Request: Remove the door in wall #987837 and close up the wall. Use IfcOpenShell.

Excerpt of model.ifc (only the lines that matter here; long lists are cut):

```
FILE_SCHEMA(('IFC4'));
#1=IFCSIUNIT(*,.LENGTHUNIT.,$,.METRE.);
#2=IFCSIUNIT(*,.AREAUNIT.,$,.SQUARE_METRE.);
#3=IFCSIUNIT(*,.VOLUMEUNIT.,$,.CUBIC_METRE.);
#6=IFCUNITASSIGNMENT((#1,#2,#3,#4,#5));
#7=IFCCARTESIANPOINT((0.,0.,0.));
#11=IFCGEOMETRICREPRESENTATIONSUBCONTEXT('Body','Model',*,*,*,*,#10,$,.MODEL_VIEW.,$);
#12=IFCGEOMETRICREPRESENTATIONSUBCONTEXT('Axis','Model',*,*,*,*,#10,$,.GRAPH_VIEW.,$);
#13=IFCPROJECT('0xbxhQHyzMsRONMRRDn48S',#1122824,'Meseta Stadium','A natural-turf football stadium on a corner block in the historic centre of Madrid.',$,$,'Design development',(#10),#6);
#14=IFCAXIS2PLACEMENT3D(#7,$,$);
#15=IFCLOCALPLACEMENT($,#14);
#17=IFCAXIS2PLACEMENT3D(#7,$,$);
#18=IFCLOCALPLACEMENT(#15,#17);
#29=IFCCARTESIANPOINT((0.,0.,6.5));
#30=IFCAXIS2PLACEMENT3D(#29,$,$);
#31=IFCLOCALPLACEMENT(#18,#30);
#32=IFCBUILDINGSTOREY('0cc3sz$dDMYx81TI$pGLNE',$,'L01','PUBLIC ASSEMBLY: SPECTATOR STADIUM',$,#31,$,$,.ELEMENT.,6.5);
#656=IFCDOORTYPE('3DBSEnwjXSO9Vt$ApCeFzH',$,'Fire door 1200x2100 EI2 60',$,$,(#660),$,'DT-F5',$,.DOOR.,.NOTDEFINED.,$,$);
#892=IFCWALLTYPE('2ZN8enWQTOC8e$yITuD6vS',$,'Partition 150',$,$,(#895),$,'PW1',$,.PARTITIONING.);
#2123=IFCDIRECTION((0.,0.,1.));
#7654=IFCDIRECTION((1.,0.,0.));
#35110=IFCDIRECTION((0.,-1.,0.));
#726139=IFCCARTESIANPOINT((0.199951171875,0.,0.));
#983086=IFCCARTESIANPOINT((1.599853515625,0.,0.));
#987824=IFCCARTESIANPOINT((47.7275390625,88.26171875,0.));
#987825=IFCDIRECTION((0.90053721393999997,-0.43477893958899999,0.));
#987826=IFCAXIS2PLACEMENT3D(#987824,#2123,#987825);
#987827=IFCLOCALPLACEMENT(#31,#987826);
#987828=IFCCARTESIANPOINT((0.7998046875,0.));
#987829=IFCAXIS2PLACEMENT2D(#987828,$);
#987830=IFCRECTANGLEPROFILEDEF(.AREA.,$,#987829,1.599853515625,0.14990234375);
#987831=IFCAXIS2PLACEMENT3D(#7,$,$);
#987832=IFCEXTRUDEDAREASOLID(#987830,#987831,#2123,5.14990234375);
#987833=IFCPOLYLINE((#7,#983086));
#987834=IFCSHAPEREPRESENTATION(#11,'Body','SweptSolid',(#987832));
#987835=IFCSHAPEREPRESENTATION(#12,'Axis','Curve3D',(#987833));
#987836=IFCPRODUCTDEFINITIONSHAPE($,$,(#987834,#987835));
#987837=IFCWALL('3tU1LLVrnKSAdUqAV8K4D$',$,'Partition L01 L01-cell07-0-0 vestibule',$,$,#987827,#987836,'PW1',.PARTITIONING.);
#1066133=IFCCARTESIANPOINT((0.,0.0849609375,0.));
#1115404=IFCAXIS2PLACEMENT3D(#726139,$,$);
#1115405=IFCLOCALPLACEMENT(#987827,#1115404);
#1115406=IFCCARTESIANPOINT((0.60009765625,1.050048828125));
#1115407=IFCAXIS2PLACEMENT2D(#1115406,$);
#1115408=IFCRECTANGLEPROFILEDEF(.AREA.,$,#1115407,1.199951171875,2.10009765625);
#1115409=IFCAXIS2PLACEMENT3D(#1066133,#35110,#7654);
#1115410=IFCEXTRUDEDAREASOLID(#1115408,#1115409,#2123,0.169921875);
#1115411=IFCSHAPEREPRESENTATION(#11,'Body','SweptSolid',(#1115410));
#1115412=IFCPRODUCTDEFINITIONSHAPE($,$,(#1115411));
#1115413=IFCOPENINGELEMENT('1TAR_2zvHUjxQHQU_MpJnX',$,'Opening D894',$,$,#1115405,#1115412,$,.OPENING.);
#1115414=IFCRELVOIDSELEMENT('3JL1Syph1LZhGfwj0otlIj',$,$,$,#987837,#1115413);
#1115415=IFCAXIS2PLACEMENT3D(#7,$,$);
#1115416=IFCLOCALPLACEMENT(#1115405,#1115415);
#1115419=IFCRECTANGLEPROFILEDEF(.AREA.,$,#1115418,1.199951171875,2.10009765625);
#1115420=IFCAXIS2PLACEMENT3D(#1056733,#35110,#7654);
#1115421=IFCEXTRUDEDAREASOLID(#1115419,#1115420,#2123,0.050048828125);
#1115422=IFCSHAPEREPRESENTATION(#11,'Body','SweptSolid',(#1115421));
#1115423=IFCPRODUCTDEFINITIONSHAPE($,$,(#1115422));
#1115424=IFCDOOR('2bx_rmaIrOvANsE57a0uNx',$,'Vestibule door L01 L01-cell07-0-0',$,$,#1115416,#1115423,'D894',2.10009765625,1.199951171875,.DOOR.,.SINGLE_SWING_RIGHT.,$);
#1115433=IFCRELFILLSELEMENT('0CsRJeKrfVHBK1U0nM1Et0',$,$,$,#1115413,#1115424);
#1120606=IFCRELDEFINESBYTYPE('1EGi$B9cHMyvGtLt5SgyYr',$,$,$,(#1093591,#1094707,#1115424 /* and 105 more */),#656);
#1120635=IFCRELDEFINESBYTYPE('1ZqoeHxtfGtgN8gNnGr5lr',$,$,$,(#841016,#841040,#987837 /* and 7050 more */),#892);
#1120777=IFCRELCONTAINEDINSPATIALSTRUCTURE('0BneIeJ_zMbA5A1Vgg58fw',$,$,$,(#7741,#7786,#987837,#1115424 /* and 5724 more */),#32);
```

```python
import ifcopenshell
import ifcopenshell.api.feature
import ifcopenshell.api.root
import ifcopenshell.geom
import ifcopenshell.util.shape

model = ifcopenshell.open("model.ifc")
settings = ifcopenshell.geom.settings()


def volume(element):
    """Net volume in cubic metres, openings subtracted."""
    shape = ifcopenshell.geom.create_shape(settings, element)
    return ifcopenshell.util.shape.get_volume(shape.geometry)


door = model.by_guid("2bx_rmaIrOvANsE57a0uNx")
opening = door.FillsVoids[0].RelatingOpeningElement
wall = opening.VoidsElements[0].RelatingBuildingElement
before = volume(wall)

ifcopenshell.api.root.remove_product(model, product=door)
ifcopenshell.api.feature.remove_feature(model, feature=opening)

after = volume(wall)

print(f"wall volume {before:.3f} -> {after:.3f} m3")

model.write("model_updated.ifc")
```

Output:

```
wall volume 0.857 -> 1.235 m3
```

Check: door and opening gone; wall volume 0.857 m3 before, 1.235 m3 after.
